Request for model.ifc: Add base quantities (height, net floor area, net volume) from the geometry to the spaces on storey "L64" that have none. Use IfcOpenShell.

First a look at what the model holds.

```python
import ifcopenshell
import ifcopenshell.util.element
import ifcopenshell.util.unit

model = ifcopenshell.open("model.ifc")
print(model.schema)
for unit_type in ("LENGTHUNIT", "AREAUNIT", "VOLUMEUNIT"):
    print(unit_type, ifcopenshell.util.unit.calculate_unit_scale(model, unit_type))
storey = next(s for s in model.by_type("IfcBuildingStorey") if s.Name == "L64")
spaces = [e for e in ifcopenshell.util.element.get_decomposition(storey) if e.is_a("IfcSpace")]
for e in sorted(spaces, key=lambda e: e.id()):
    print(e.id(), e.is_a(), e.Name, list(ifcopenshell.util.element.get_psets(e, qtos_only=True)), sep=" | ")
```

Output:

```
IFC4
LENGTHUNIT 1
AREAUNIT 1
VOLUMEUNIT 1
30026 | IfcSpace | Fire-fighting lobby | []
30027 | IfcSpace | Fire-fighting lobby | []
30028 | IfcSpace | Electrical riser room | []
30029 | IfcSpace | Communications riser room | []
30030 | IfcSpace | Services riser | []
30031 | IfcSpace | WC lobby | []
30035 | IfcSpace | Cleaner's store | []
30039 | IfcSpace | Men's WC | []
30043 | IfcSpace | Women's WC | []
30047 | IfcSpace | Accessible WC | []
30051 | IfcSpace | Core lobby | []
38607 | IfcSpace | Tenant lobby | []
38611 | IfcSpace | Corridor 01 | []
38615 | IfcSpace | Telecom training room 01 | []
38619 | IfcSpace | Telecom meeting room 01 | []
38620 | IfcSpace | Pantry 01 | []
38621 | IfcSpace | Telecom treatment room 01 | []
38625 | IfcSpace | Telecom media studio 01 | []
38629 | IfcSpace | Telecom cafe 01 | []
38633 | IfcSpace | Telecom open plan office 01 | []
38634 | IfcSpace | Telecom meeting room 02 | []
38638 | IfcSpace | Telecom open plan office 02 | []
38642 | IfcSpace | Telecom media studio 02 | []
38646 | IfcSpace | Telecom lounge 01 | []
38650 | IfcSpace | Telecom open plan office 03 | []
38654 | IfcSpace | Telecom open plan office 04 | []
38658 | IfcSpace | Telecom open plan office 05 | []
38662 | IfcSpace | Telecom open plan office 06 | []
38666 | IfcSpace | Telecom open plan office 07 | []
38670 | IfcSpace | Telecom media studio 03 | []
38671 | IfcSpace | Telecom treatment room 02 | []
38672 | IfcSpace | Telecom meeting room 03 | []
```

```python
import ifcopenshell
import ifcopenshell.api.pset
import ifcopenshell.geom
import ifcopenshell.util.element
import ifcopenshell.util.shape
import ifcopenshell.util.unit

model = ifcopenshell.open("model.ifc")
unit_scale = ifcopenshell.util.unit.calculate_unit_scale(model)
area_scale = ifcopenshell.util.unit.calculate_unit_scale(model, "AREAUNIT")
volume_scale = ifcopenshell.util.unit.calculate_unit_scale(model, "VOLUMEUNIT")
settings = ifcopenshell.geom.settings()

storey = next(s for s in model.by_type("IfcBuildingStorey") if s.Name == "L64")
spaces = [e for e in ifcopenshell.util.element.get_decomposition(storey) if e.is_a("IfcSpace")]

for e in sorted(spaces, key=lambda e: e.id()):
    if ifcopenshell.util.element.get_psets(e, qtos_only=True, should_inherit=False):
        continue
    # Geometry comes back in metres, in the element's own axes.
    shape = ifcopenshell.geom.create_shape(settings, e)
    values = {
        "Height": ifcopenshell.util.shape.get_z(shape.geometry) / unit_scale,
        "NetFloorArea": ifcopenshell.util.shape.get_footprint_area(shape.geometry) / area_scale,
        "NetVolume": ifcopenshell.util.shape.get_volume(shape.geometry) / volume_scale,
    }
    qto = ifcopenshell.api.pset.add_qto(model, product=e, name="Qto_SpaceBaseQuantities")
    ifcopenshell.api.pset.edit_qto(model, qto=qto, properties=values)
    print(e.id(), {k: round(v, 3) for k, v in values.items()})

model.write("model_edited.ifc")
```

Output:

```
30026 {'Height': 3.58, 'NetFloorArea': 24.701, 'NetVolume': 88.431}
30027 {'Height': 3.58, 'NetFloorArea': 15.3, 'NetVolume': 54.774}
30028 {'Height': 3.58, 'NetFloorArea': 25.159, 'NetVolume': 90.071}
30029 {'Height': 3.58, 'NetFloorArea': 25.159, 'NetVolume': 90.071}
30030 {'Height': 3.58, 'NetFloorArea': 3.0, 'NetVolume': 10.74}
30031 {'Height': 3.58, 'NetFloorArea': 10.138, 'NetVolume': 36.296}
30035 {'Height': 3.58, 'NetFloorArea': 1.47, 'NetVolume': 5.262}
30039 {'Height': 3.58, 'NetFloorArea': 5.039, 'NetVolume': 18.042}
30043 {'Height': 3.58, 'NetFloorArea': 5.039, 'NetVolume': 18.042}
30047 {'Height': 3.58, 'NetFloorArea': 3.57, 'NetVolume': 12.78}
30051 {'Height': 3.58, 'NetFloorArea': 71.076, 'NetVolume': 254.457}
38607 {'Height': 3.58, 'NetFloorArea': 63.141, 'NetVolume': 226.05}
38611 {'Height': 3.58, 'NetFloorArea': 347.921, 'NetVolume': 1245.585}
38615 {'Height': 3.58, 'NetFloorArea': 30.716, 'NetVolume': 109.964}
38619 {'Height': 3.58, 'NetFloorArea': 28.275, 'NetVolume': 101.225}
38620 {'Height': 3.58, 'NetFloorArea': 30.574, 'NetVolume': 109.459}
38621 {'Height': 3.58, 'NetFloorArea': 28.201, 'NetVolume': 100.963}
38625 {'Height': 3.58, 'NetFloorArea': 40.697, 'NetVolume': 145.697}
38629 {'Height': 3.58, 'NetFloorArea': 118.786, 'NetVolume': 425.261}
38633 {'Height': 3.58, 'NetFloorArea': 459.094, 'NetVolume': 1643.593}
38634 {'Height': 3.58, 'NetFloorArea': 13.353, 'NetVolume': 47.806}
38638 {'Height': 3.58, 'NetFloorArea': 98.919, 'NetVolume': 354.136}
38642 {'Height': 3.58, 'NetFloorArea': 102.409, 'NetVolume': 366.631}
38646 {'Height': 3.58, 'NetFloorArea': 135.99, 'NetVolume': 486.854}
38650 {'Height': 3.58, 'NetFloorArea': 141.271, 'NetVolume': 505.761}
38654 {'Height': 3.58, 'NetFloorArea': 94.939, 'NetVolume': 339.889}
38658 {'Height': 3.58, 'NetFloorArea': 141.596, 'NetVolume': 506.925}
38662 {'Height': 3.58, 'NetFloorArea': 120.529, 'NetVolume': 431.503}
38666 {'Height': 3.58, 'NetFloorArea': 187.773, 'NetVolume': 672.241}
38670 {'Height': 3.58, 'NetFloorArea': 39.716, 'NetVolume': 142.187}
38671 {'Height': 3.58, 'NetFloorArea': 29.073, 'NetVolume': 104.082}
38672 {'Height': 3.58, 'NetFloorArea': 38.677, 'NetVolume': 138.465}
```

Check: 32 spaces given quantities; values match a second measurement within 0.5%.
